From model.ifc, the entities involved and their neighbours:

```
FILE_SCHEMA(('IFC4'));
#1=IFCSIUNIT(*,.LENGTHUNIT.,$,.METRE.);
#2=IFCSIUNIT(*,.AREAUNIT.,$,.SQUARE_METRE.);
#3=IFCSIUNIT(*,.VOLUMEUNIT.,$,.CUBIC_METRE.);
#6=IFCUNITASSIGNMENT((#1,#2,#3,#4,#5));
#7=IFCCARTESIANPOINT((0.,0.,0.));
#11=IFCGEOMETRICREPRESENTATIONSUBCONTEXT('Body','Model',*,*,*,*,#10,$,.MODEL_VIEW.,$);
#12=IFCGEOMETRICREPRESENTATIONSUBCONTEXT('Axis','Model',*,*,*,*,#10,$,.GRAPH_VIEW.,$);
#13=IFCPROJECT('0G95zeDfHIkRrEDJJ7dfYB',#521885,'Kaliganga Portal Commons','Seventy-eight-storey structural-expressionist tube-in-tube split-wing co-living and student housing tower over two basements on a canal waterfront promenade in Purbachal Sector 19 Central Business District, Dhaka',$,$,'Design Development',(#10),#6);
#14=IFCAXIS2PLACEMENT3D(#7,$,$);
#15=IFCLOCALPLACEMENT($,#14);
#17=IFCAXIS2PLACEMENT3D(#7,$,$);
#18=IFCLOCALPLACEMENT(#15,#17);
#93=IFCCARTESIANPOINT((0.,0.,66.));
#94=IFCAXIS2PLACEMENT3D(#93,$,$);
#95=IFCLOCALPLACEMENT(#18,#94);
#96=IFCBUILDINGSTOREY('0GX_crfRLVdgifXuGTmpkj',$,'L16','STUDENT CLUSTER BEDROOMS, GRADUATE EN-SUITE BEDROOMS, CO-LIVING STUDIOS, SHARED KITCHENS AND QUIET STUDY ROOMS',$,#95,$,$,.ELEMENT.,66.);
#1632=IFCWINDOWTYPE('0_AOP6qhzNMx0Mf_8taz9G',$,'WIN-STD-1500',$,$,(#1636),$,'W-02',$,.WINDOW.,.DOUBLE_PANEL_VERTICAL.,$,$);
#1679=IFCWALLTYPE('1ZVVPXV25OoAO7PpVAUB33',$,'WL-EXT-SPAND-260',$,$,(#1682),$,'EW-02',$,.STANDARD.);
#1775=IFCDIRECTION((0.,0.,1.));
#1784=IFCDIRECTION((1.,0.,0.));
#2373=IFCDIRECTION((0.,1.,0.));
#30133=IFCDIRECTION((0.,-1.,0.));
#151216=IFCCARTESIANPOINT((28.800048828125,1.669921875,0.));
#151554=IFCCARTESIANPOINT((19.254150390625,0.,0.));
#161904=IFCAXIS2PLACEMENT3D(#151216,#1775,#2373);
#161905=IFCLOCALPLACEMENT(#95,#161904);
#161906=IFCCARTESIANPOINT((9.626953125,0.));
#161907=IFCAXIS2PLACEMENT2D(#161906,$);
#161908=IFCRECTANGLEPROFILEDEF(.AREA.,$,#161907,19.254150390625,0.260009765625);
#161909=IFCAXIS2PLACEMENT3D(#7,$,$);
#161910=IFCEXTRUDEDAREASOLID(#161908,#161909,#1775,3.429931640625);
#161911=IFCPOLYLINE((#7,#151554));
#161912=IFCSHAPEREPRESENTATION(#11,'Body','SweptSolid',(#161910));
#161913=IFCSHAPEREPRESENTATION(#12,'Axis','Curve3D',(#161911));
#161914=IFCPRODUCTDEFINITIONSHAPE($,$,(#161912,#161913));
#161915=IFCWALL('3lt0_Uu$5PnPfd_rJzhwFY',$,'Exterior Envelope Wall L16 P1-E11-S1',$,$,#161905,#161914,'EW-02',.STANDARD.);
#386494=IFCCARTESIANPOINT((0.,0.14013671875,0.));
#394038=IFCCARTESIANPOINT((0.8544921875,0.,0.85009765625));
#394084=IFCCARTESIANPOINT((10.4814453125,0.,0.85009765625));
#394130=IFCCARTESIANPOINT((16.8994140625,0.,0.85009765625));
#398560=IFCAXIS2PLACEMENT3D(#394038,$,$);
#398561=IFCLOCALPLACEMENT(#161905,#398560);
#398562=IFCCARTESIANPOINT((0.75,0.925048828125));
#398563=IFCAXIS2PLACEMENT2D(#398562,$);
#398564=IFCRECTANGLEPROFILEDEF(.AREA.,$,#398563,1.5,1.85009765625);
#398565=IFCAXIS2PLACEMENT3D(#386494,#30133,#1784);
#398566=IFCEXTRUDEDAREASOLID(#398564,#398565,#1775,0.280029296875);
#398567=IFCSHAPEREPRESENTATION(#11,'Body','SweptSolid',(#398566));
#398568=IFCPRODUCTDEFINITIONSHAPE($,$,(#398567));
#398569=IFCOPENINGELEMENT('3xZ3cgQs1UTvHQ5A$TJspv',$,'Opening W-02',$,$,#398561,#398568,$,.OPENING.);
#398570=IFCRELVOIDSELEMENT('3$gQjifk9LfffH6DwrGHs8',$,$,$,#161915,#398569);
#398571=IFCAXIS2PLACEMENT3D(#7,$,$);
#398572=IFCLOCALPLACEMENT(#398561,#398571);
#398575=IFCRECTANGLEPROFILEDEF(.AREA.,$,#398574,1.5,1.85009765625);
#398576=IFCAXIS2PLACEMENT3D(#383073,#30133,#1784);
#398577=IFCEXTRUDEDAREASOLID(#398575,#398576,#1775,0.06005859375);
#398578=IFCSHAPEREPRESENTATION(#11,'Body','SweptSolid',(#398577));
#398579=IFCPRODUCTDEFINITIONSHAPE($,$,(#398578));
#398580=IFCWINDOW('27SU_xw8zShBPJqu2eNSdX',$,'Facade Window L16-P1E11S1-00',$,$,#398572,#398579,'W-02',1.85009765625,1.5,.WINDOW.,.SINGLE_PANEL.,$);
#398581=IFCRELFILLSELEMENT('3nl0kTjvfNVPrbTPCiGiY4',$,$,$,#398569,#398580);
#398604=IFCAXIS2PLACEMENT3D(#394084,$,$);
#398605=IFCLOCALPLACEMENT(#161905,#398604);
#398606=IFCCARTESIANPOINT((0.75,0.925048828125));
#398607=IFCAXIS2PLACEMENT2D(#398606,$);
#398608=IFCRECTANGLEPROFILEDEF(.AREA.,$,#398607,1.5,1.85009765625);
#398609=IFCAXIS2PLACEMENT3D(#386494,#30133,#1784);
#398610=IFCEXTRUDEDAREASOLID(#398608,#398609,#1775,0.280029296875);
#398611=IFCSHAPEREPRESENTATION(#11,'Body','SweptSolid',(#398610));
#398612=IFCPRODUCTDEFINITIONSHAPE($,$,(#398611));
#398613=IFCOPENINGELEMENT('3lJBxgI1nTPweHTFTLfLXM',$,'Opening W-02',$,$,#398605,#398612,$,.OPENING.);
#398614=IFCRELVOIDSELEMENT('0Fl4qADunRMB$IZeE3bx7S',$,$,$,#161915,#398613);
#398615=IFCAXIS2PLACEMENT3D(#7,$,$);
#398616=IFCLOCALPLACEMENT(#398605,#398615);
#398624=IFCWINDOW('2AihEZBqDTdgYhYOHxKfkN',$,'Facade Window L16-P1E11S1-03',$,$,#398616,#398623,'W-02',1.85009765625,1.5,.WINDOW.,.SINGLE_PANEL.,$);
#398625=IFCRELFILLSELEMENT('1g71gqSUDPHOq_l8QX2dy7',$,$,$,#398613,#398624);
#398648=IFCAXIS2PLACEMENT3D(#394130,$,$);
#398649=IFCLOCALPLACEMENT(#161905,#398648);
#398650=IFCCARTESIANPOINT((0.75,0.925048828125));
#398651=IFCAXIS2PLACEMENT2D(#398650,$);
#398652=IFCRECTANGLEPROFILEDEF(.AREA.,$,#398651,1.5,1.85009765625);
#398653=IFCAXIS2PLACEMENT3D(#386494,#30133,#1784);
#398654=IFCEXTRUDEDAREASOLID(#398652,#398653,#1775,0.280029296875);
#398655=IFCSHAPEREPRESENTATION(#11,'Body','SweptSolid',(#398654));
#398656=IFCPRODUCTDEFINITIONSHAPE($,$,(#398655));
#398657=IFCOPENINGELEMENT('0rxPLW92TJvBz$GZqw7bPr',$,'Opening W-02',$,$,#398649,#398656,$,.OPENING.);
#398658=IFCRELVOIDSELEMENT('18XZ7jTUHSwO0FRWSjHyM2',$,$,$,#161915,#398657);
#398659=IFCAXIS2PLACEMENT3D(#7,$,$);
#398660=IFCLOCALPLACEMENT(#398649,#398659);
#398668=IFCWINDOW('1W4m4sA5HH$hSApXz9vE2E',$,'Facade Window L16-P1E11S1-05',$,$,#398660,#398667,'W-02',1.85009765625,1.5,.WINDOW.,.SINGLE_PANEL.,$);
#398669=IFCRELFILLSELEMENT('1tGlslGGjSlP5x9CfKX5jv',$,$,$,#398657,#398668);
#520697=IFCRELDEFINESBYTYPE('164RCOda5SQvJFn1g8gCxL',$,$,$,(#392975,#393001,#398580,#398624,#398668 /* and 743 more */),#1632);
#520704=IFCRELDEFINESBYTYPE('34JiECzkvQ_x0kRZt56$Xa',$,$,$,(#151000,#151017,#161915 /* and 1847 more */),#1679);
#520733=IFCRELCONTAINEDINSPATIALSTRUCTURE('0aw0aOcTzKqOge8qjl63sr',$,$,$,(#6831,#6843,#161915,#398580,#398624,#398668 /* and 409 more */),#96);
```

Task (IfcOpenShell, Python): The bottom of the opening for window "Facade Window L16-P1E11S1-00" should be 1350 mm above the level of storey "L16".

```python
import numpy as np
import ifcopenshell
import ifcopenshell.api.geometry
import ifcopenshell.geom
import ifcopenshell.util.element
import ifcopenshell.util.placement
import ifcopenshell.util.shape
import ifcopenshell.util.unit

model = ifcopenshell.open("model.ifc")
unit_scale = ifcopenshell.util.unit.calculate_unit_scale(model)

window = model.by_guid("27SU_xw8zShBPJqu2eNSdX")
opening = window.FillsVoids[0].RelatingOpeningElement
storey = ifcopenshell.util.element.get_container(window, ifc_class="IfcBuildingStorey")
level = ifcopenshell.util.placement.get_local_placement(storey.ObjectPlacement)[2, 3]

# The opening's origin need not be at the sill, so measure its lowest point.
shape = ifcopenshell.geom.create_shape(ifcopenshell.geom.settings(), opening)
bottom = ifcopenshell.util.shape.get_shape_bottom_elevation(shape, shape.geometry) / unit_scale
dz = level + 1.35 - bottom

shift = np.array([0.0, 0.0, dz])
# The window is placed relative to its opening, so it follows when the opening moves.
matrix = ifcopenshell.util.placement.get_local_placement(opening.ObjectPlacement)
matrix[:3, 3] += shift
ifcopenshell.api.geometry.edit_object_placement(
    model, product=opening, matrix=matrix, is_si=False, should_transform_children=True
)

print(f"moved by {dz * unit_scale:+.3f} m")

model.write("model_rev.ifc")
```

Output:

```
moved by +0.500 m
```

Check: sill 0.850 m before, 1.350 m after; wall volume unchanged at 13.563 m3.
